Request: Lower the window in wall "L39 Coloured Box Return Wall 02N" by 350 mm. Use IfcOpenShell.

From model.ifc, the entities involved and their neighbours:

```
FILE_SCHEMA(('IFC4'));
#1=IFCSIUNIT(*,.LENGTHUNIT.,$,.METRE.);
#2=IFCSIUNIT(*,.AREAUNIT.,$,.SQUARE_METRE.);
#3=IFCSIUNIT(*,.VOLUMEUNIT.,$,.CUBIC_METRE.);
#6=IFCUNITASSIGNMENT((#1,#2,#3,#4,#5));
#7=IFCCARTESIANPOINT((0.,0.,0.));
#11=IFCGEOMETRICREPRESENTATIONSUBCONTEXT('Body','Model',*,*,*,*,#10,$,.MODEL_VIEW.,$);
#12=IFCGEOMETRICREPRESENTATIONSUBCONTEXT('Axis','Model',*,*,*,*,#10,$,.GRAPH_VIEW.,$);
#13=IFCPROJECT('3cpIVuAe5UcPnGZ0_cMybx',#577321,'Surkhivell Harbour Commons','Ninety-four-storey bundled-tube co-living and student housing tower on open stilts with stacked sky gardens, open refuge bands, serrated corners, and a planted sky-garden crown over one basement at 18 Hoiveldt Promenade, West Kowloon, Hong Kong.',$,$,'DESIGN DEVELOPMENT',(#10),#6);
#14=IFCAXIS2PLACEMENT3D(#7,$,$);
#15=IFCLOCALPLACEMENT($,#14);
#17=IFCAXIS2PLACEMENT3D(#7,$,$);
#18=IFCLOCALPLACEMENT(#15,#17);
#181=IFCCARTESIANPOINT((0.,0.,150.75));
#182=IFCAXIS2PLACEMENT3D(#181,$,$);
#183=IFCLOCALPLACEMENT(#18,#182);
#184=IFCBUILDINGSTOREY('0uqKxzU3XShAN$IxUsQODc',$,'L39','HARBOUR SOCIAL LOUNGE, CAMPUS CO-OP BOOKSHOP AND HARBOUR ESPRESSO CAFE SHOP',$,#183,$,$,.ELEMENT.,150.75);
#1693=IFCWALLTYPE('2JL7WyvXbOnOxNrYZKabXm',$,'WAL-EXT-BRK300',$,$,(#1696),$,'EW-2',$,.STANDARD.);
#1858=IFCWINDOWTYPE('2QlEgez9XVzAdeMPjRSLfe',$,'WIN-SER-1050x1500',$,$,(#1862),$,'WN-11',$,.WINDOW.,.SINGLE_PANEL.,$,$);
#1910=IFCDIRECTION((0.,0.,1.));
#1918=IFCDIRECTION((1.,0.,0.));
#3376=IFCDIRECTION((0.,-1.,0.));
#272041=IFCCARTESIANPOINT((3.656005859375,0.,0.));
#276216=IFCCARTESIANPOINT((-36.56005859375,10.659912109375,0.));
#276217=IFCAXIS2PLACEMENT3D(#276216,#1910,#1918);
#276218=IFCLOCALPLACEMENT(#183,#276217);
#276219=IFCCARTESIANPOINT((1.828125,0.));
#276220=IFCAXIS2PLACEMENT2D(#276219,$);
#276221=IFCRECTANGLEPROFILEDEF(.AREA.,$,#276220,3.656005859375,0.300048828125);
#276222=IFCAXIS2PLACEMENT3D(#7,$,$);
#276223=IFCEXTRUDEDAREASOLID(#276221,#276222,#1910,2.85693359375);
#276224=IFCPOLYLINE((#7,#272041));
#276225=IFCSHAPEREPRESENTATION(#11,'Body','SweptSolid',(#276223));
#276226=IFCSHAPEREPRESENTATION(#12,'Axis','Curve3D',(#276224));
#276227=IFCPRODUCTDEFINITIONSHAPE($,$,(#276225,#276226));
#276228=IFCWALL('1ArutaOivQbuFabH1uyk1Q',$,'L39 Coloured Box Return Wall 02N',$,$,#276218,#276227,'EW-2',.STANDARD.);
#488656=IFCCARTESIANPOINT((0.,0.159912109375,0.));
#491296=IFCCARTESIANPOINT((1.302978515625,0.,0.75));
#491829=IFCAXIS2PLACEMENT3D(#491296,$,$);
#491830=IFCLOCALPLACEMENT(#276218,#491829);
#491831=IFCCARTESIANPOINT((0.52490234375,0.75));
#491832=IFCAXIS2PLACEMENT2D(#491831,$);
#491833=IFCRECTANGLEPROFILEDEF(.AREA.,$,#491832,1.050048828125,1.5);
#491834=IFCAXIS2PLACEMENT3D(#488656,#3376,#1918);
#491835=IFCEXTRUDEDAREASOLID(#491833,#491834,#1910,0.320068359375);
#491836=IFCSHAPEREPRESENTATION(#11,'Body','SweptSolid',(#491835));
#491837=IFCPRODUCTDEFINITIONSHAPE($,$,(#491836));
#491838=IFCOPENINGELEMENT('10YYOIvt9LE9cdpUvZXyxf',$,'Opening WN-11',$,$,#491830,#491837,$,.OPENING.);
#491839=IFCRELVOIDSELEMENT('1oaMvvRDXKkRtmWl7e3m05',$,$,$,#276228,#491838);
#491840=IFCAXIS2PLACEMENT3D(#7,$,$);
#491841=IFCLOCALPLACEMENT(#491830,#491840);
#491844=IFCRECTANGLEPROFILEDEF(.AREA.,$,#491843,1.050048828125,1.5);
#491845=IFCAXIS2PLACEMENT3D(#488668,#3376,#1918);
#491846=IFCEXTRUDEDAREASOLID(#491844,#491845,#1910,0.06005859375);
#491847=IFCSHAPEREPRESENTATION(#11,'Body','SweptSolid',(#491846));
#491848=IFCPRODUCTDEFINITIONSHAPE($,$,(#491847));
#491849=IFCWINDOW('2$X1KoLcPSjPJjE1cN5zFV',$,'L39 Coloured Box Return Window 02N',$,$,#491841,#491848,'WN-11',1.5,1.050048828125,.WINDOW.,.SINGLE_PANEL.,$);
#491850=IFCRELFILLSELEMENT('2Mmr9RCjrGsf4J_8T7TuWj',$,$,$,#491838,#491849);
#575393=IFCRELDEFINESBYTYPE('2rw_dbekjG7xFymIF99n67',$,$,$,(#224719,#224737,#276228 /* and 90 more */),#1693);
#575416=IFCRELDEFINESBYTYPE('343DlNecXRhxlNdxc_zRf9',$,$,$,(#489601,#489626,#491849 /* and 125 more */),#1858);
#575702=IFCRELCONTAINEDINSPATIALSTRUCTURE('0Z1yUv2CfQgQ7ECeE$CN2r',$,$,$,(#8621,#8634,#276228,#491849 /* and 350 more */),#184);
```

```python
import numpy as np
import ifcopenshell
import ifcopenshell.api.geometry
import ifcopenshell.util.placement
import ifcopenshell.util.unit

model = ifcopenshell.open("model.ifc")
unit_scale = ifcopenshell.util.unit.calculate_unit_scale(model)

window = model.by_guid("2$X1KoLcPSjPJjE1cN5zFV")
opening = window.FillsVoids[0].RelatingOpeningElement
dz = -0.35

shift = np.array([0.0, 0.0, dz])
# The window is placed relative to its opening, so it follows when the opening moves.
matrix = ifcopenshell.util.placement.get_local_placement(opening.ObjectPlacement)
matrix[:3, 3] += shift
ifcopenshell.api.geometry.edit_object_placement(
    model, product=opening, matrix=matrix, is_si=False, should_transform_children=True
)

print(f"moved by {dz * unit_scale:+.3f} m")

model.write("model_rev.ifc")
```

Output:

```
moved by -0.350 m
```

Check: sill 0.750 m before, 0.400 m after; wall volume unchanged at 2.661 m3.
